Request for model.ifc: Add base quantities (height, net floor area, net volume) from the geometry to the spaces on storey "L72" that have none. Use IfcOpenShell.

First a look at what the model holds.

```python
import ifcopenshell
import ifcopenshell.util.element
import ifcopenshell.util.unit

model = ifcopenshell.open("model.ifc")
print(model.schema)
for unit_type in ("LENGTHUNIT", "AREAUNIT", "VOLUMEUNIT"):
    print(unit_type, ifcopenshell.util.unit.calculate_unit_scale(model, unit_type))
storey = next(s for s in model.by_type("IfcBuildingStorey") if s.Name == "L72")
spaces = [e for e in ifcopenshell.util.element.get_decomposition(storey) if e.is_a("IfcSpace")]
for e in sorted(spaces, key=lambda e: e.id()):
    print(e.id(), e.is_a(), e.Name, list(ifcopenshell.util.element.get_psets(e, qtos_only=True)), sep=" | ")
```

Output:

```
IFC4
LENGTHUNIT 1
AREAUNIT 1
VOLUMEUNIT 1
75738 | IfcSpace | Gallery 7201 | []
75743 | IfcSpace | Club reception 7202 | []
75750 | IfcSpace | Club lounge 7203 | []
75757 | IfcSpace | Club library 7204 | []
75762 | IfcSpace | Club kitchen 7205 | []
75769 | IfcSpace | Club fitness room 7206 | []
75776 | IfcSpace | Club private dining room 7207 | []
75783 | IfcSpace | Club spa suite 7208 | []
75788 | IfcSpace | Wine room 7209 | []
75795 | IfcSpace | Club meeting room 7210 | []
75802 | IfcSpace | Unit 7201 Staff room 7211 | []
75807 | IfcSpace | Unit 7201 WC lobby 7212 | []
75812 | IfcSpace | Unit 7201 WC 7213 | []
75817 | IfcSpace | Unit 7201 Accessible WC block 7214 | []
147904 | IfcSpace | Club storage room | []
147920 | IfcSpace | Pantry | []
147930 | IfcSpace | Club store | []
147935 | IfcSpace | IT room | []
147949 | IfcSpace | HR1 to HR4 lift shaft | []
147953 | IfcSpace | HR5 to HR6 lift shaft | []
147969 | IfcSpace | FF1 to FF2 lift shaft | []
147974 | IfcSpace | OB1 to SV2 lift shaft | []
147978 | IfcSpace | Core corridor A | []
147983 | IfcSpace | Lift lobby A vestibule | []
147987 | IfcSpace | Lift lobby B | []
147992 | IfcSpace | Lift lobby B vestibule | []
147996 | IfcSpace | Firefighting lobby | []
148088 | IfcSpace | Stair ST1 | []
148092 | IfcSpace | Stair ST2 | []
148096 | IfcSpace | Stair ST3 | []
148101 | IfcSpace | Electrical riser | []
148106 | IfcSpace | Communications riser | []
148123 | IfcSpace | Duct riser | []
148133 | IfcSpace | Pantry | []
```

```python
import ifcopenshell
import ifcopenshell.api.pset
import ifcopenshell.geom
import ifcopenshell.util.element
import ifcopenshell.util.shape
import ifcopenshell.util.unit

model = ifcopenshell.open("model.ifc")
unit_scale = ifcopenshell.util.unit.calculate_unit_scale(model)
area_scale = ifcopenshell.util.unit.calculate_unit_scale(model, "AREAUNIT")
volume_scale = ifcopenshell.util.unit.calculate_unit_scale(model, "VOLUMEUNIT")
settings = ifcopenshell.geom.settings()

storey = next(s for s in model.by_type("IfcBuildingStorey") if s.Name == "L72")
spaces = [e for e in ifcopenshell.util.element.get_decomposition(storey) if e.is_a("IfcSpace")]

for e in sorted(spaces, key=lambda e: e.id()):
    if ifcopenshell.util.element.get_psets(e, qtos_only=True, should_inherit=False):
        continue
    # Geometry comes back in metres, in the element's own axes.
    shape = ifcopenshell.geom.create_shape(settings, e)
    values = {
        "Height": ifcopenshell.util.shape.get_z(shape.geometry) / unit_scale,
        "NetFloorArea": ifcopenshell.util.shape.get_footprint_area(shape.geometry) / area_scale,
        "NetVolume": ifcopenshell.util.shape.get_volume(shape.geometry) / volume_scale,
    }
    qto = ifcopenshell.api.pset.add_qto(model, product=e, name="Qto_SpaceBaseQuantities")
    ifcopenshell.api.pset.edit_qto(model, qto=qto, properties=values)
    print(e.id(), {k: round(v, 3) for k, v in values.items()})

model.write("model_v2.ifc")
```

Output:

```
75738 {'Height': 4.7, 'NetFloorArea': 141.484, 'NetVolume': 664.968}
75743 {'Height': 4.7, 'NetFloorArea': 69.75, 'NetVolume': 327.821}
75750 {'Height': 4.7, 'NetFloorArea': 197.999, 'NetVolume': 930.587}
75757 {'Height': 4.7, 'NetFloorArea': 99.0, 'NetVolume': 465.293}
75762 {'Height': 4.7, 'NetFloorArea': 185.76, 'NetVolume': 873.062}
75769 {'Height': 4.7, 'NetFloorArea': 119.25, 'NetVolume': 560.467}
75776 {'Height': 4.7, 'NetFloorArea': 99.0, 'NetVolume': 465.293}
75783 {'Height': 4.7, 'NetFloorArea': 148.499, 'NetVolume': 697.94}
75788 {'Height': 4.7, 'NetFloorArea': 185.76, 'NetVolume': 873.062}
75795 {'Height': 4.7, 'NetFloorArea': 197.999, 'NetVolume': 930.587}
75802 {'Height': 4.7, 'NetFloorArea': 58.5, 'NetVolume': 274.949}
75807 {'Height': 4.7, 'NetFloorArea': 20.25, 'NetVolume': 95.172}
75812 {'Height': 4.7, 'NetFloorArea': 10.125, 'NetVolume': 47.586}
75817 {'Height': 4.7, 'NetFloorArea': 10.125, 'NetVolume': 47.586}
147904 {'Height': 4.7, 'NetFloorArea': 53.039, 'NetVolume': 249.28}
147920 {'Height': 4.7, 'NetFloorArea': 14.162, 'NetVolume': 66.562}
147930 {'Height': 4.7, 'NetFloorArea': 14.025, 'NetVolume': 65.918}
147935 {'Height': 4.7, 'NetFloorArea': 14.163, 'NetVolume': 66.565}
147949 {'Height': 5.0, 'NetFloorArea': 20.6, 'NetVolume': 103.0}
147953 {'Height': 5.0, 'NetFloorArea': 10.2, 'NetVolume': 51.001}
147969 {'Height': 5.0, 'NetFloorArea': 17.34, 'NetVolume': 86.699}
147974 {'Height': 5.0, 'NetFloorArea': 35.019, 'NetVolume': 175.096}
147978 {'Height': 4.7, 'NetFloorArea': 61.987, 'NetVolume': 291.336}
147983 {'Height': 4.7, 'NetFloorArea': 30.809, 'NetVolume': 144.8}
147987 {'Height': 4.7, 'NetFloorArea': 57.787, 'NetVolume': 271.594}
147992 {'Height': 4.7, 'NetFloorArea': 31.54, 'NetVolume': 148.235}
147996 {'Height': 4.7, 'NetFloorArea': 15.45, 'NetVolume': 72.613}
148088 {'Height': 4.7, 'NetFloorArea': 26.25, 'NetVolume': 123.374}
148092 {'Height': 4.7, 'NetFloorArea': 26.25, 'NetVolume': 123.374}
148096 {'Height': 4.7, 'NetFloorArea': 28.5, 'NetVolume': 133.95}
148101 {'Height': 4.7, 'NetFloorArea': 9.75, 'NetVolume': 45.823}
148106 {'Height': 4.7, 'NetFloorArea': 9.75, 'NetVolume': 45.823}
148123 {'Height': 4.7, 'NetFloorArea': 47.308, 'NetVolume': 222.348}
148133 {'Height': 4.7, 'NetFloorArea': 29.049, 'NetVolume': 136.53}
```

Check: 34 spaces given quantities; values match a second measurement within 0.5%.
